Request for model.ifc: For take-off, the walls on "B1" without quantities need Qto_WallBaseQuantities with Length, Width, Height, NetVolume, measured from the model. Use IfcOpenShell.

First a look at what the model holds.

```python
import ifcopenshell
import ifcopenshell.util.element
import ifcopenshell.util.unit

model = ifcopenshell.open("model.ifc")
print(model.schema)
for unit_type in ("LENGTHUNIT", "AREAUNIT", "VOLUMEUNIT"):
    print(unit_type, ifcopenshell.util.unit.calculate_unit_scale(model, unit_type))
storey = next(s for s in model.by_type("IfcBuildingStorey") if s.Name == "B1")
walls = [e for e in ifcopenshell.util.element.get_decomposition(storey) if e.is_a("IfcWall")]
for e in sorted(walls, key=lambda e: e.id()):
    print(e.id(), e.is_a(), e.Name, list(ifcopenshell.util.element.get_psets(e, qtos_only=True)), sep=" | ")
```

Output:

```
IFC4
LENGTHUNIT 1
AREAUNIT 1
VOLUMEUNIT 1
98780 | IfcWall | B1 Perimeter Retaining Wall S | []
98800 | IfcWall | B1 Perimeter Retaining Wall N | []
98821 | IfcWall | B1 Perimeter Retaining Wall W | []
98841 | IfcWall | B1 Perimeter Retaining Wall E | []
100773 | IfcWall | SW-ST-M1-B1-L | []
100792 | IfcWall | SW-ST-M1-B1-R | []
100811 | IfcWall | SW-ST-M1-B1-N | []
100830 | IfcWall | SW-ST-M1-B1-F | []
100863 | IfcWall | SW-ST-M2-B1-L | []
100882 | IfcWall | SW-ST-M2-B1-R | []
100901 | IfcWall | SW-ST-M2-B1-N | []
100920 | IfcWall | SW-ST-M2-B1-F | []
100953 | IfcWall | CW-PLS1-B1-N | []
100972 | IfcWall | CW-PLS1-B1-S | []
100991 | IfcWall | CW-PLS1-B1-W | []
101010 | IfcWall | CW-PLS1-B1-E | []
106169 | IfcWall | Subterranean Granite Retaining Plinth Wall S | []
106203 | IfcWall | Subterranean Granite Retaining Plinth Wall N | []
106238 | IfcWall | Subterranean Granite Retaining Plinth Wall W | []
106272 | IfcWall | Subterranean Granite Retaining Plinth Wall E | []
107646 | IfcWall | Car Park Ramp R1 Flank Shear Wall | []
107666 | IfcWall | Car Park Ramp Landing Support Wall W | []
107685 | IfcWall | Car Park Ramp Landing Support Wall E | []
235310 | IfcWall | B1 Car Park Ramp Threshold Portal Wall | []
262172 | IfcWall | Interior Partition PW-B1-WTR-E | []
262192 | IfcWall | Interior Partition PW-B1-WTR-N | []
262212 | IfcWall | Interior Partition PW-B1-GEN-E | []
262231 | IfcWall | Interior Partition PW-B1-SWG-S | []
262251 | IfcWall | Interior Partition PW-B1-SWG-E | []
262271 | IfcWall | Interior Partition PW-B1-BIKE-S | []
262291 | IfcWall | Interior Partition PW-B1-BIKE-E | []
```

```python
import ifcopenshell
import ifcopenshell.api.pset
import ifcopenshell.geom
import ifcopenshell.util.element
import ifcopenshell.util.shape
import ifcopenshell.util.unit

model = ifcopenshell.open("model.ifc")
unit_scale = ifcopenshell.util.unit.calculate_unit_scale(model)
volume_scale = ifcopenshell.util.unit.calculate_unit_scale(model, "VOLUMEUNIT")
settings = ifcopenshell.geom.settings()

storey = next(s for s in model.by_type("IfcBuildingStorey") if s.Name == "B1")
walls = [e for e in ifcopenshell.util.element.get_decomposition(storey) if e.is_a("IfcWall")]

for e in sorted(walls, key=lambda e: e.id()):
    if ifcopenshell.util.element.get_psets(e, qtos_only=True, should_inherit=False):
        continue
    # Geometry comes back in metres, in the element's own axes.
    shape = ifcopenshell.geom.create_shape(settings, e)
    values = {
        "Length": ifcopenshell.util.shape.get_x(shape.geometry) / unit_scale,
        "Width": ifcopenshell.util.shape.get_y(shape.geometry) / unit_scale,
        "Height": ifcopenshell.util.shape.get_z(shape.geometry) / unit_scale,
        "NetVolume": ifcopenshell.util.shape.get_volume(shape.geometry) / volume_scale,
    }
    qto = ifcopenshell.api.pset.add_qto(model, product=e, name="Qto_WallBaseQuantities")
    ifcopenshell.api.pset.edit_qto(model, qto=qto, properties=values)
    print(e.id(), {k: round(v, 3) for k, v in values.items()})

model.write("model_updated.ifc")
```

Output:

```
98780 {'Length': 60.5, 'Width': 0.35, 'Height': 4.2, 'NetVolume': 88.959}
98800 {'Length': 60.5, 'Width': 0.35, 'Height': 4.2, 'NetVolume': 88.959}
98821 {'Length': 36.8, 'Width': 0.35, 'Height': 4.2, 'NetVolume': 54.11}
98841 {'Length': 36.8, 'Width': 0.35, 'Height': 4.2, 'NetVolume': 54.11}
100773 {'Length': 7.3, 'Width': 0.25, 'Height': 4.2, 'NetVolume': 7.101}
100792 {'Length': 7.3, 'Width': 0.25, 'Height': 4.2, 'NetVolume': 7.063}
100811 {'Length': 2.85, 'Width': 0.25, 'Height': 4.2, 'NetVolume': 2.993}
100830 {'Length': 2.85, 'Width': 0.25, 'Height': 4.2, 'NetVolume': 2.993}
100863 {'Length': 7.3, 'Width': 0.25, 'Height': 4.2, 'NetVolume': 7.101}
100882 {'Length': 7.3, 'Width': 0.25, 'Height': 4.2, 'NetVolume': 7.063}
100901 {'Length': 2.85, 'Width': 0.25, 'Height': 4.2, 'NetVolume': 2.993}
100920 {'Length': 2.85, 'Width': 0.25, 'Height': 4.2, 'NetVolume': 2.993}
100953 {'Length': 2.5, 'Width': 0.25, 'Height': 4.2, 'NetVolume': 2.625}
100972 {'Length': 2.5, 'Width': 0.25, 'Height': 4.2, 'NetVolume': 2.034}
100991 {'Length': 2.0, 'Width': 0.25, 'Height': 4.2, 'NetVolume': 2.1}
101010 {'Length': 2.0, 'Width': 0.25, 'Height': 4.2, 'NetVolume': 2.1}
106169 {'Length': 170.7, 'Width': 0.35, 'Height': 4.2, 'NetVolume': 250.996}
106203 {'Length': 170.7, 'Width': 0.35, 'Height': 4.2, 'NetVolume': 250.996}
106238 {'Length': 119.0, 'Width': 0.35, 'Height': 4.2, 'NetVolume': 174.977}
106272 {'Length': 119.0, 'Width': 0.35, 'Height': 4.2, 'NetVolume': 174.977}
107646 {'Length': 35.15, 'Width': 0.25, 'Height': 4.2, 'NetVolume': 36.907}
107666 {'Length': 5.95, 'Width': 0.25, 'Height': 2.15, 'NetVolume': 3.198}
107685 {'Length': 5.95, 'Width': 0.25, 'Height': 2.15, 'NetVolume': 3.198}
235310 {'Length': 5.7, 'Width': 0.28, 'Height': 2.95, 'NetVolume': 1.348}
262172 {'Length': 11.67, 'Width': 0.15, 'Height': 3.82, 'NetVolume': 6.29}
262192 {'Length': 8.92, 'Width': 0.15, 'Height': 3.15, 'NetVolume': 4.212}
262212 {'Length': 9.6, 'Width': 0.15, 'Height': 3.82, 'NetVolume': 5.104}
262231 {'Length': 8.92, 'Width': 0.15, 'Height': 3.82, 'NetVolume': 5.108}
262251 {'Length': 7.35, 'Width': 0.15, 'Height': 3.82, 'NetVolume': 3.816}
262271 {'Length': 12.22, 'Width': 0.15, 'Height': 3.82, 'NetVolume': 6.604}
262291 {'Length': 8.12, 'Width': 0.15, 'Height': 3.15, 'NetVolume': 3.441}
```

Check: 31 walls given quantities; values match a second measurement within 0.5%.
